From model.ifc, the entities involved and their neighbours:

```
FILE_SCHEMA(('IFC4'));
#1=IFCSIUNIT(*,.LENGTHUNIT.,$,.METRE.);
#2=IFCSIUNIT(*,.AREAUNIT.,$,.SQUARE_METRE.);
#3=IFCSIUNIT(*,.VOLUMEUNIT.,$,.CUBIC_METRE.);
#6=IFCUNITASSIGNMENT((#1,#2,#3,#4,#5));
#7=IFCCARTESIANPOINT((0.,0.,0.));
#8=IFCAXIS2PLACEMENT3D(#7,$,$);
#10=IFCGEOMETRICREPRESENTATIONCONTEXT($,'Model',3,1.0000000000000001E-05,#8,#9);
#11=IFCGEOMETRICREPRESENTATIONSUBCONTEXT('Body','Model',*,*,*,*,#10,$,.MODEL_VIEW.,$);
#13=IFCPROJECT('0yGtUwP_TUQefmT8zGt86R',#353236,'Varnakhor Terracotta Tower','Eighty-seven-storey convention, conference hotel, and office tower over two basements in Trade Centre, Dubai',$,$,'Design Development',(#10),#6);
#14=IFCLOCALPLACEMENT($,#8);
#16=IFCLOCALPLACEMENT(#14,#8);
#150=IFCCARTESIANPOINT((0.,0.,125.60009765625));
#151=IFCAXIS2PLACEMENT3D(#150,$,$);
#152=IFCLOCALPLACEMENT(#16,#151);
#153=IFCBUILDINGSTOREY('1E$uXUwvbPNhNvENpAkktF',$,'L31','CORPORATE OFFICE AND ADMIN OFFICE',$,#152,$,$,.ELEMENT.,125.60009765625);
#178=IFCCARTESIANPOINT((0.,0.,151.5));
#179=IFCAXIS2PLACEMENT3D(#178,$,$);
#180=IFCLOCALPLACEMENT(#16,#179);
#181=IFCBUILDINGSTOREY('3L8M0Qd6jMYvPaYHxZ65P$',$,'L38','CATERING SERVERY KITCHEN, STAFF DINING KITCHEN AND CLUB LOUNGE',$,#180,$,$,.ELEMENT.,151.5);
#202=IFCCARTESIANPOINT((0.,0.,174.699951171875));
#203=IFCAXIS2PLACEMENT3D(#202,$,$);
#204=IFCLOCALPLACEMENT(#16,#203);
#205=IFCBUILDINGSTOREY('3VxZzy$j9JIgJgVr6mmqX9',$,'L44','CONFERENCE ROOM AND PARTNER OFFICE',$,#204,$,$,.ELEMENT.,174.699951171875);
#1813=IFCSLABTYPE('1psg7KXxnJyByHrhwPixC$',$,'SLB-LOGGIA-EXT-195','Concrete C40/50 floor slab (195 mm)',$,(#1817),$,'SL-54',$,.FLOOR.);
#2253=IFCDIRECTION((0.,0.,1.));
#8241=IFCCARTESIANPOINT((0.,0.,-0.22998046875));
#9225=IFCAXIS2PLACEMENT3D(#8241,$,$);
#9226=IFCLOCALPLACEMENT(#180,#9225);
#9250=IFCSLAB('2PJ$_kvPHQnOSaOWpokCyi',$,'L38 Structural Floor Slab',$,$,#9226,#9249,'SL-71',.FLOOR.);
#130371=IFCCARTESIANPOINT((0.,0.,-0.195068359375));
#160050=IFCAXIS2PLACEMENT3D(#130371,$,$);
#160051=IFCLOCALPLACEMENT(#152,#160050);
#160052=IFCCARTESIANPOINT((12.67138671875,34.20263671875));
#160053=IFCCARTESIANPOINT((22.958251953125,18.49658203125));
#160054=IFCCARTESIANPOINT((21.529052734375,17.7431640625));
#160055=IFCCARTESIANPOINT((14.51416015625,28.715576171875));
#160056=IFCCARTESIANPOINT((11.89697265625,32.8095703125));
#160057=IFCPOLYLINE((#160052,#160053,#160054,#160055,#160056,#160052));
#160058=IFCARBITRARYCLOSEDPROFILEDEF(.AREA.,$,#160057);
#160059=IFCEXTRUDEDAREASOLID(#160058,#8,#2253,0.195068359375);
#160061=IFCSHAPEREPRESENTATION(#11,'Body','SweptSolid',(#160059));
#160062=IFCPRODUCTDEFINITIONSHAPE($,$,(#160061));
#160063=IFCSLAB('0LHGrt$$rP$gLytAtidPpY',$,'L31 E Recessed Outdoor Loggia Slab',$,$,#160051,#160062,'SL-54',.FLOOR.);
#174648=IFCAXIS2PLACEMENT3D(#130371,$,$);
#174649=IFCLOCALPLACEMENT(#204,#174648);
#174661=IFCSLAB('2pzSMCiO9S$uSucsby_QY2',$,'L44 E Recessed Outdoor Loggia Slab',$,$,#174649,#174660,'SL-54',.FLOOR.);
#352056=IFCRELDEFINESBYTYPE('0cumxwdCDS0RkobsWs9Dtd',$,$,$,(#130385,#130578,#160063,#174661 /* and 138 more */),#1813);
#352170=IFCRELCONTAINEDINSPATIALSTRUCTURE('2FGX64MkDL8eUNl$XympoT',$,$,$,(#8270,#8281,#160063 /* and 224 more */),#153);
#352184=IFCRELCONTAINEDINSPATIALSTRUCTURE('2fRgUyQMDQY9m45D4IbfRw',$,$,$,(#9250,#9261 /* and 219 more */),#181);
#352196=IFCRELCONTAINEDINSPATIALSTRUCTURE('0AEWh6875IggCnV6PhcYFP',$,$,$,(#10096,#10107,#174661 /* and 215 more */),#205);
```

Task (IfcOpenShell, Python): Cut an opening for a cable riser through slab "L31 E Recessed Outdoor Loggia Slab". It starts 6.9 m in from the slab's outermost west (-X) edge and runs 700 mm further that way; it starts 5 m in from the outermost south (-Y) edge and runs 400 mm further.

```python
import numpy as np
import ifcopenshell
import ifcopenshell.api.feature
import ifcopenshell.api.geometry
import ifcopenshell.api.root
import ifcopenshell.geom
import ifcopenshell.util.placement
import ifcopenshell.util.representation
import ifcopenshell.util.shape
import ifcopenshell.util.unit

model = ifcopenshell.open("model.ifc")
unit_scale = ifcopenshell.util.unit.calculate_unit_scale(model)
settings = ifcopenshell.geom.settings()


def volume(element):
    """Net volume in cubic metres, openings subtracted."""
    shape = ifcopenshell.geom.create_shape(settings, element)
    return ifcopenshell.util.shape.get_volume(shape.geometry)


slab = model.by_guid("0LHGrt$$rP$gLytAtidPpY")
before = volume(slab)

# Extent in the slab's own axes, in metres. The edges named are its -X and -Y sides.
slab_shape = ifcopenshell.geom.create_shape(settings, slab)
vertices = ifcopenshell.util.shape.get_vertices(slab_shape.geometry)
x_min, y_min, bottom = vertices.min(axis=0)
top = vertices[:, 2].max()

opening = ifcopenshell.api.root.create_entity(model, ifc_class="IfcOpeningElement", name="Cable riser opening", predefined_type="OPENING")
context = ifcopenshell.util.representation.get_context(model, "Model", "Body", "MODEL_VIEW")
width, depth = 0.7, 0.4
outline = [(0.0, 0.0), (width, 0.0), (width, depth), (0.0, depth), (0.0, 0.0)]
# Overshoot both faces by 50 mm so the cut is clean.
shape = ifcopenshell.api.geometry.add_slab_representation(
    model, context=context, depth=top - bottom + 0.1, polyline=outline
)
ifcopenshell.api.geometry.assign_representation(model, product=opening, representation=shape)

matrix = ifcopenshell.util.placement.get_local_placement(slab.ObjectPlacement)
matrix[:, 3] = matrix @ np.append(np.array([x_min + 6.9, y_min + 5, bottom - 0.05]) / unit_scale, 1.0)
ifcopenshell.api.geometry.edit_object_placement(model, product=opening, matrix=matrix, is_si=False)
ifcopenshell.api.feature.add_feature(model, feature=opening, element=slab)

after = volume(slab)

print(f"slab volume {before:.3f} -> {after:.3f} m3")

model.write("model_rev.ifc")
```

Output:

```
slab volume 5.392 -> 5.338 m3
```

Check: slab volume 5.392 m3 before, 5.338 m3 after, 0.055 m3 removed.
